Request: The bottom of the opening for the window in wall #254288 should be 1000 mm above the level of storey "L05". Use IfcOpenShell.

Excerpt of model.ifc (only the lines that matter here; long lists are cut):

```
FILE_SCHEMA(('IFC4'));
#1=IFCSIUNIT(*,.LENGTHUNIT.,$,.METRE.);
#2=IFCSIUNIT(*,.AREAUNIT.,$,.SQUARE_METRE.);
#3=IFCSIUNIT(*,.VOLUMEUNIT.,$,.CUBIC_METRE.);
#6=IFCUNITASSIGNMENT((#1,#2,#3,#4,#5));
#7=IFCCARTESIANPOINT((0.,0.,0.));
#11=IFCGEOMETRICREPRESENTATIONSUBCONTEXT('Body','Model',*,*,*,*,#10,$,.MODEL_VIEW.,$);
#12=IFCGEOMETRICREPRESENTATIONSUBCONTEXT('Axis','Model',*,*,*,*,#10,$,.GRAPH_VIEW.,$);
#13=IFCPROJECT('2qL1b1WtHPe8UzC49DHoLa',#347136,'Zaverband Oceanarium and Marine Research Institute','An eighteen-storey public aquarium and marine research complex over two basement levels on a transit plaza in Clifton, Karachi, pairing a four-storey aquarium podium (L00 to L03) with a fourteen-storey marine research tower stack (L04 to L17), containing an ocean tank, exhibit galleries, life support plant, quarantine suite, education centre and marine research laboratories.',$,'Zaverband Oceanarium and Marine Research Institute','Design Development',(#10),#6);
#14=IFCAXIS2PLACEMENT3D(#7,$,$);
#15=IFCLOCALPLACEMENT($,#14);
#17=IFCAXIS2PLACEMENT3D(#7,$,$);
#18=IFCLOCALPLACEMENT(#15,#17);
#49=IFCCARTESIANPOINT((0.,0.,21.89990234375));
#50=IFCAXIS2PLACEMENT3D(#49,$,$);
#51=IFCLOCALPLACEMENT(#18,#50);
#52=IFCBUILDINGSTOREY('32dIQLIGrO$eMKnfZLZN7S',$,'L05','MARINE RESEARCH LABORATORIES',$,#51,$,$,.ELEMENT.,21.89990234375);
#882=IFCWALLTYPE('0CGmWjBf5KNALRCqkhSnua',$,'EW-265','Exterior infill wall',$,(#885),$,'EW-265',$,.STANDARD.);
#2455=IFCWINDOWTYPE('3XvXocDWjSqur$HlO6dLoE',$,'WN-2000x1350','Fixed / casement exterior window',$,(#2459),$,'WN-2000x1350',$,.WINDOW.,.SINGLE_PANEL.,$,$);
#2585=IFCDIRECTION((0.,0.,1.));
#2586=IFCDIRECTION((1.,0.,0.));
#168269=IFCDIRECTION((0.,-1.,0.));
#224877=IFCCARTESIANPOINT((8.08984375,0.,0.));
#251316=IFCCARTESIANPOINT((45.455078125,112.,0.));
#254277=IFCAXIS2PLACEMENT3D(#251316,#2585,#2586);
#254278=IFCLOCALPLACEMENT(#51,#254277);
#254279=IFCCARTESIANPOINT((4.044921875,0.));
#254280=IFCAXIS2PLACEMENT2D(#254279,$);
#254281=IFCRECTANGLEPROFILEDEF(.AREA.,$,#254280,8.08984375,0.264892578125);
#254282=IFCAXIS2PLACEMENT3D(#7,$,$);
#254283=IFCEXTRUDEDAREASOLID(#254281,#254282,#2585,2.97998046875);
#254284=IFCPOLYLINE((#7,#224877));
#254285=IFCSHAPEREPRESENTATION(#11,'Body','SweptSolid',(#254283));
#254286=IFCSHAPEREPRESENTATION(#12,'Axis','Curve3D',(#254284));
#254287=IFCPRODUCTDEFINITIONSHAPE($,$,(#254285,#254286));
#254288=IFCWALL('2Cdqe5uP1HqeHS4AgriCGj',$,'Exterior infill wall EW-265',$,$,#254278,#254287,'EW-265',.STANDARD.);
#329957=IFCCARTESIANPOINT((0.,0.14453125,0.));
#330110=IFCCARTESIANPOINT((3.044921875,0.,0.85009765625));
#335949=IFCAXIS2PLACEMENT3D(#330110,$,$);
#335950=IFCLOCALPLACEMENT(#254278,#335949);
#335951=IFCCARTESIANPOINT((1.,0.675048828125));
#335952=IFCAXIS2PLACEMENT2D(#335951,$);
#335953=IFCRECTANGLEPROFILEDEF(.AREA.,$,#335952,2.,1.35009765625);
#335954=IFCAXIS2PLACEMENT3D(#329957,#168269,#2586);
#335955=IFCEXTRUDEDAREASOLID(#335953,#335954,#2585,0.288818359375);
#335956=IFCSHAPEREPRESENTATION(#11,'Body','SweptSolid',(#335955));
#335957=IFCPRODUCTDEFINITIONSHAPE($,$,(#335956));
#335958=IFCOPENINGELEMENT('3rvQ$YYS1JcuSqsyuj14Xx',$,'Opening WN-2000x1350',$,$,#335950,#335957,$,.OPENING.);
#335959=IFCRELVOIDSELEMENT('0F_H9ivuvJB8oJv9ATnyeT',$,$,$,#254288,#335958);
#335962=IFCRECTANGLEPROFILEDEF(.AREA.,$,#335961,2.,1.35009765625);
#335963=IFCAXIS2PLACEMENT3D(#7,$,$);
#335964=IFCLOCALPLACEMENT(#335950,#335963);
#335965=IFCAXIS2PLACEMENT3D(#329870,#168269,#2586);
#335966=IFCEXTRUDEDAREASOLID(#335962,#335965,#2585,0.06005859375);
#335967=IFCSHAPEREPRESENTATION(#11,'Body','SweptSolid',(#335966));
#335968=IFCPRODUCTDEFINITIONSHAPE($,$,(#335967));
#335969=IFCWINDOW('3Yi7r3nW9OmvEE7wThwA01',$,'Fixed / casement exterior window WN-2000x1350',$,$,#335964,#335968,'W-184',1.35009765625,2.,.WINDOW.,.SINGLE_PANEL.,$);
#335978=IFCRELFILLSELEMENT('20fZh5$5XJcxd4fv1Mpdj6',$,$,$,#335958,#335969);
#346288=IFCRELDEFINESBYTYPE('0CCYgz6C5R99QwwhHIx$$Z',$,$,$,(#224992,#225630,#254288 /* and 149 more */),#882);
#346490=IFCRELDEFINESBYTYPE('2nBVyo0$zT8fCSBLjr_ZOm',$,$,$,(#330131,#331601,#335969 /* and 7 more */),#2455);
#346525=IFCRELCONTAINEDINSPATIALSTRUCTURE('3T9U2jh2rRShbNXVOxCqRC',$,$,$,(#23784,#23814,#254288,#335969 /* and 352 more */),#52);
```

```python
import numpy as np
import ifcopenshell
import ifcopenshell.api.geometry
import ifcopenshell.geom
import ifcopenshell.util.element
import ifcopenshell.util.placement
import ifcopenshell.util.shape
import ifcopenshell.util.unit

model = ifcopenshell.open("model.ifc")
unit_scale = ifcopenshell.util.unit.calculate_unit_scale(model)

window = model.by_id(335969)
opening = window.FillsVoids[0].RelatingOpeningElement
storey = ifcopenshell.util.element.get_container(window, ifc_class="IfcBuildingStorey")
level = ifcopenshell.util.placement.get_local_placement(storey.ObjectPlacement)[2, 3]

# The opening's origin need not be at the sill, so measure its lowest point.
shape = ifcopenshell.geom.create_shape(ifcopenshell.geom.settings(), opening)
bottom = ifcopenshell.util.shape.get_shape_bottom_elevation(shape, shape.geometry) / unit_scale
dz = level + 1 / unit_scale - bottom

shift = np.array([0.0, 0.0, dz])
# The window is placed relative to its opening, so it follows when the opening moves.
matrix = ifcopenshell.util.placement.get_local_placement(opening.ObjectPlacement)
matrix[:3, 3] += shift
ifcopenshell.api.geometry.edit_object_placement(
    model, product=opening, matrix=matrix, is_si=False, should_transform_children=True
)

print(f"moved by {dz * unit_scale:+.3f} m")

model.write("model_rev.ifc")
```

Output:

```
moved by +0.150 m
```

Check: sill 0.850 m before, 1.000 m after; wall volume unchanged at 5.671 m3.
